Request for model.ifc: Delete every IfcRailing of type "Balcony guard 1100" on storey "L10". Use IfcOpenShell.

First a look at what the model holds.

```python
import ifcopenshell
import ifcopenshell.util.element

model = ifcopenshell.open("model.ifc")
print(model.schema)
storey = next(s for s in model.by_type("IfcBuildingStorey") if s.Name == "L10")
railings = [e for e in ifcopenshell.util.element.get_decomposition(storey) if e.is_a("IfcRailing")]
seen = {}
for e in railings:
    element_type = ifcopenshell.util.element.get_type(e)
    name = element_type.Name if element_type not in (None, e) else None
    seen[name] = seen.get(name, 0) + 1
for name, count in sorted(seen.items(), key=str):
    print(count, "x", name)
```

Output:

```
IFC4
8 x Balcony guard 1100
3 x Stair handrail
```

```python
import ifcopenshell
import ifcopenshell.api.root
import ifcopenshell.util.element

model = ifcopenshell.open("model.ifc")

storey = next(s for s in model.by_type("IfcBuildingStorey") if s.Name == "L10")
railings = [e for e in ifcopenshell.util.element.get_decomposition(storey) if e.is_a("IfcRailing")]
targets = [e for e in railings if (t := ifcopenshell.util.element.get_type(e)) not in (None, e) and t.Name == "Balcony guard 1100"]

for e in targets:
    ifcopenshell.api.root.remove_product(model, product=e)
print(len(targets), "removed")

model.write("model_v2.ifc")
```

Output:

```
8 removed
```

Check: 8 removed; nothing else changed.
